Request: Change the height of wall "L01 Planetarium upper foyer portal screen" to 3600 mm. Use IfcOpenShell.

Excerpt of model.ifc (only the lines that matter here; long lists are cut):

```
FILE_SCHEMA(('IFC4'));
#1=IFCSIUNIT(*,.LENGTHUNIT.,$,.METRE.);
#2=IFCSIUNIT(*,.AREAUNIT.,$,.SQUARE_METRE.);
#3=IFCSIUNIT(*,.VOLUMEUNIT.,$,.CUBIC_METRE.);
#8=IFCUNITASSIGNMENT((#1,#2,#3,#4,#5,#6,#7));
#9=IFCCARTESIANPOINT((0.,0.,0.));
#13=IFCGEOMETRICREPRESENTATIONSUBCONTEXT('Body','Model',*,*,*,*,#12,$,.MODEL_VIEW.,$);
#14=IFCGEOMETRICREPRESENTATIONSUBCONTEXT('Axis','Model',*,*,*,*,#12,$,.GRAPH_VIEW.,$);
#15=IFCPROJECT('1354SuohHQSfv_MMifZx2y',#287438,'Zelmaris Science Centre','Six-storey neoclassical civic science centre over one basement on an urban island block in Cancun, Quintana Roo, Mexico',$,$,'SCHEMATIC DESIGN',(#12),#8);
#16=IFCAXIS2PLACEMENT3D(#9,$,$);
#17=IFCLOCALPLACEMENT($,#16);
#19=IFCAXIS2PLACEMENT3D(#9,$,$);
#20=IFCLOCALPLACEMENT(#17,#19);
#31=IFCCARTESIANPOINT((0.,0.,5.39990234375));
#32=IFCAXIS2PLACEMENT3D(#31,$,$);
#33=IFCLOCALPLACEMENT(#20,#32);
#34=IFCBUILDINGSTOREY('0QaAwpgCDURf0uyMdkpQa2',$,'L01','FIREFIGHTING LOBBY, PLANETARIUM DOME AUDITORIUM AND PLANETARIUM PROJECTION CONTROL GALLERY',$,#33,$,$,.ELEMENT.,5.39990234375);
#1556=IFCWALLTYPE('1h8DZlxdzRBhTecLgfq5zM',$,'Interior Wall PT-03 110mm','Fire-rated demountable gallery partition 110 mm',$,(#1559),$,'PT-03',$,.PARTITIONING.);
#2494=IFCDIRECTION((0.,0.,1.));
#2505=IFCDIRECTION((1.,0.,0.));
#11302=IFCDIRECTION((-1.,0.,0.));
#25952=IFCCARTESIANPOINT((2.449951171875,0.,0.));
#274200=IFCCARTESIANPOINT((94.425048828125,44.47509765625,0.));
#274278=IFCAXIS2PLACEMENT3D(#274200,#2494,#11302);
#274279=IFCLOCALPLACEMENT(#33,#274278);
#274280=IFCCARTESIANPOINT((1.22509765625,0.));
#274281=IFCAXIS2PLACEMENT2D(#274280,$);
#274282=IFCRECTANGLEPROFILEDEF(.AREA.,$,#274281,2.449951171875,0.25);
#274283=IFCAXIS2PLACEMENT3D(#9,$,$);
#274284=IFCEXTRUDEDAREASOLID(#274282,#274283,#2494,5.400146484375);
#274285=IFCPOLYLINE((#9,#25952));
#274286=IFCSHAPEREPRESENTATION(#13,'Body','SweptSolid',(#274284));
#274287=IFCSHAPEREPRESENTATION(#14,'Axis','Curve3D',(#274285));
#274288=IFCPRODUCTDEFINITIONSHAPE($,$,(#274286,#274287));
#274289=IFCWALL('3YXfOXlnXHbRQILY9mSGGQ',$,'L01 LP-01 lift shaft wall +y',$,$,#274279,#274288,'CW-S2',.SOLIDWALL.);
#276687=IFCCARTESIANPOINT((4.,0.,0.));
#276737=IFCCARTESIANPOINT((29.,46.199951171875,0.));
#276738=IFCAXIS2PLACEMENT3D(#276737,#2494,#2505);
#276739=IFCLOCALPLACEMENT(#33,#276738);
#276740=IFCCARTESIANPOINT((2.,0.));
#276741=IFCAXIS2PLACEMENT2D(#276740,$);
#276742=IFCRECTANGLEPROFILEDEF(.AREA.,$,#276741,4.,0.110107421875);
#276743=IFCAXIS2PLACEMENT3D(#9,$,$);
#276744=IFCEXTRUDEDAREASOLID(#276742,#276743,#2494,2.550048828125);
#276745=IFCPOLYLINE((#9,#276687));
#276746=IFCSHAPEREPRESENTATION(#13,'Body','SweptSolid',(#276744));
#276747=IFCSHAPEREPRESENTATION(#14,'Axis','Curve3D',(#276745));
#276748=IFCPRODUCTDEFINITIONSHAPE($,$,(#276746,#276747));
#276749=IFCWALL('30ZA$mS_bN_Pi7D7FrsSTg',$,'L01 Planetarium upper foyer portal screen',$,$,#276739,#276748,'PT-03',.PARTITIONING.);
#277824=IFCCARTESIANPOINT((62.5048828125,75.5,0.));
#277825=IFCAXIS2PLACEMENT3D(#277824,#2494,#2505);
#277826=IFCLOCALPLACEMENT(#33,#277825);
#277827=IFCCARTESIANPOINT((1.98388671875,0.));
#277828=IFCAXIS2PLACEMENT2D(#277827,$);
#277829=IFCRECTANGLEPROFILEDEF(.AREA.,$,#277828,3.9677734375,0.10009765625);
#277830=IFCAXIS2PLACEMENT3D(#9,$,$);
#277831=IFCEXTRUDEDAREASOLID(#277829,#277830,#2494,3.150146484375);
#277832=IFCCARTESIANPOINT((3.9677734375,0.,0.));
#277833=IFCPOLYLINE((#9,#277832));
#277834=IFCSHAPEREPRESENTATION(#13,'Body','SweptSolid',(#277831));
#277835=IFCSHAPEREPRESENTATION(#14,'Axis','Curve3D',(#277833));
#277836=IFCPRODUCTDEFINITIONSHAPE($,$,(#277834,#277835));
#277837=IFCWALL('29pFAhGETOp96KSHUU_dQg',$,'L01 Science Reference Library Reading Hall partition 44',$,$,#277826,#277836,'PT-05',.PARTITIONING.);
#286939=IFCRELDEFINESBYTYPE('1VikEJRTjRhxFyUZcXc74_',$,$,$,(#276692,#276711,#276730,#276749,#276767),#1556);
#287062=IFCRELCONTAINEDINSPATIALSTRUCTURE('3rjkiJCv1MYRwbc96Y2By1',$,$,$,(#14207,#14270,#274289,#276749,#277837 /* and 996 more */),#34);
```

```python
import ifcopenshell
import ifcopenshell.geom
import ifcopenshell.util.representation
import ifcopenshell.util.shape

model = ifcopenshell.open("model.ifc")
settings = ifcopenshell.geom.settings()


def volume(element):
    """Net volume in cubic metres, openings subtracted."""
    shape = ifcopenshell.geom.create_shape(settings, element)
    return ifcopenshell.util.shape.get_volume(shape.geometry)


wall = model.by_id(276749)
before = volume(wall)

body = ifcopenshell.util.representation.get_representation(wall, "Model", "Body")
solid = body.Items[0]
old_height = solid.Depth
solid.Depth = 3.6
after = volume(wall)

print(f"height {old_height:g} -> {solid.Depth:g}, volume {before:.3f} -> {after:.3f} m3")

model.write("model_edited.ifc")
```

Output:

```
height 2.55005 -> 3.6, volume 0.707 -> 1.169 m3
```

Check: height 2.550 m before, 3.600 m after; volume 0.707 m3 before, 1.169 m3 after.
